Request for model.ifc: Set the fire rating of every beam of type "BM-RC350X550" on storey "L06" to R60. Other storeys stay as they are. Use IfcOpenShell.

First a look at what the model holds.

```python
import ifcopenshell
import ifcopenshell.util.element

model = ifcopenshell.open("model.ifc")
print(model.schema)
storey = next(s for s in model.by_type("IfcBuildingStorey") if s.Name == "L06")
beams = [e for e in ifcopenshell.util.element.get_decomposition(storey) if e.is_a("IfcBeam")]
seen = {}
for e in beams:
    element_type = ifcopenshell.util.element.get_type(e)
    key = (element_type.Name if element_type != e and element_type else None, ifcopenshell.util.element.get_pset(e, "Pset_BeamCommon", "FireRating"))
    seen[key] = seen.get(key, 0) + 1
for (name, value), count in sorted(seen.items(), key=str):
    print(count, "x", name, "|", value)
```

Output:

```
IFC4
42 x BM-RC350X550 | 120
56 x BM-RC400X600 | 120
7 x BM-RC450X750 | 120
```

```python
import ifcopenshell
import ifcopenshell.api.pset
import ifcopenshell.util.element

model = ifcopenshell.open("model.ifc")

storey = next(s for s in model.by_type("IfcBuildingStorey") if s.Name == "L06")
beams = [e for e in ifcopenshell.util.element.get_decomposition(storey) if e.is_a("IfcBeam")]

count = 0
for e in beams:
    element_type = ifcopenshell.util.element.get_type(e)
    if element_type in (None, e) or element_type.Name != "BM-RC350X550":
        continue
    # add_pset returns the element's existing set when there is one.
    pset = ifcopenshell.api.pset.add_pset(model, product=e, name="Pset_BeamCommon")
    ifcopenshell.api.pset.edit_pset(model, pset=pset, properties={"FireRating": "R60"})
    count += 1

print(count, "beams updated")

model.write("model-out.ifc")
```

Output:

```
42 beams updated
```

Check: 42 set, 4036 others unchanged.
